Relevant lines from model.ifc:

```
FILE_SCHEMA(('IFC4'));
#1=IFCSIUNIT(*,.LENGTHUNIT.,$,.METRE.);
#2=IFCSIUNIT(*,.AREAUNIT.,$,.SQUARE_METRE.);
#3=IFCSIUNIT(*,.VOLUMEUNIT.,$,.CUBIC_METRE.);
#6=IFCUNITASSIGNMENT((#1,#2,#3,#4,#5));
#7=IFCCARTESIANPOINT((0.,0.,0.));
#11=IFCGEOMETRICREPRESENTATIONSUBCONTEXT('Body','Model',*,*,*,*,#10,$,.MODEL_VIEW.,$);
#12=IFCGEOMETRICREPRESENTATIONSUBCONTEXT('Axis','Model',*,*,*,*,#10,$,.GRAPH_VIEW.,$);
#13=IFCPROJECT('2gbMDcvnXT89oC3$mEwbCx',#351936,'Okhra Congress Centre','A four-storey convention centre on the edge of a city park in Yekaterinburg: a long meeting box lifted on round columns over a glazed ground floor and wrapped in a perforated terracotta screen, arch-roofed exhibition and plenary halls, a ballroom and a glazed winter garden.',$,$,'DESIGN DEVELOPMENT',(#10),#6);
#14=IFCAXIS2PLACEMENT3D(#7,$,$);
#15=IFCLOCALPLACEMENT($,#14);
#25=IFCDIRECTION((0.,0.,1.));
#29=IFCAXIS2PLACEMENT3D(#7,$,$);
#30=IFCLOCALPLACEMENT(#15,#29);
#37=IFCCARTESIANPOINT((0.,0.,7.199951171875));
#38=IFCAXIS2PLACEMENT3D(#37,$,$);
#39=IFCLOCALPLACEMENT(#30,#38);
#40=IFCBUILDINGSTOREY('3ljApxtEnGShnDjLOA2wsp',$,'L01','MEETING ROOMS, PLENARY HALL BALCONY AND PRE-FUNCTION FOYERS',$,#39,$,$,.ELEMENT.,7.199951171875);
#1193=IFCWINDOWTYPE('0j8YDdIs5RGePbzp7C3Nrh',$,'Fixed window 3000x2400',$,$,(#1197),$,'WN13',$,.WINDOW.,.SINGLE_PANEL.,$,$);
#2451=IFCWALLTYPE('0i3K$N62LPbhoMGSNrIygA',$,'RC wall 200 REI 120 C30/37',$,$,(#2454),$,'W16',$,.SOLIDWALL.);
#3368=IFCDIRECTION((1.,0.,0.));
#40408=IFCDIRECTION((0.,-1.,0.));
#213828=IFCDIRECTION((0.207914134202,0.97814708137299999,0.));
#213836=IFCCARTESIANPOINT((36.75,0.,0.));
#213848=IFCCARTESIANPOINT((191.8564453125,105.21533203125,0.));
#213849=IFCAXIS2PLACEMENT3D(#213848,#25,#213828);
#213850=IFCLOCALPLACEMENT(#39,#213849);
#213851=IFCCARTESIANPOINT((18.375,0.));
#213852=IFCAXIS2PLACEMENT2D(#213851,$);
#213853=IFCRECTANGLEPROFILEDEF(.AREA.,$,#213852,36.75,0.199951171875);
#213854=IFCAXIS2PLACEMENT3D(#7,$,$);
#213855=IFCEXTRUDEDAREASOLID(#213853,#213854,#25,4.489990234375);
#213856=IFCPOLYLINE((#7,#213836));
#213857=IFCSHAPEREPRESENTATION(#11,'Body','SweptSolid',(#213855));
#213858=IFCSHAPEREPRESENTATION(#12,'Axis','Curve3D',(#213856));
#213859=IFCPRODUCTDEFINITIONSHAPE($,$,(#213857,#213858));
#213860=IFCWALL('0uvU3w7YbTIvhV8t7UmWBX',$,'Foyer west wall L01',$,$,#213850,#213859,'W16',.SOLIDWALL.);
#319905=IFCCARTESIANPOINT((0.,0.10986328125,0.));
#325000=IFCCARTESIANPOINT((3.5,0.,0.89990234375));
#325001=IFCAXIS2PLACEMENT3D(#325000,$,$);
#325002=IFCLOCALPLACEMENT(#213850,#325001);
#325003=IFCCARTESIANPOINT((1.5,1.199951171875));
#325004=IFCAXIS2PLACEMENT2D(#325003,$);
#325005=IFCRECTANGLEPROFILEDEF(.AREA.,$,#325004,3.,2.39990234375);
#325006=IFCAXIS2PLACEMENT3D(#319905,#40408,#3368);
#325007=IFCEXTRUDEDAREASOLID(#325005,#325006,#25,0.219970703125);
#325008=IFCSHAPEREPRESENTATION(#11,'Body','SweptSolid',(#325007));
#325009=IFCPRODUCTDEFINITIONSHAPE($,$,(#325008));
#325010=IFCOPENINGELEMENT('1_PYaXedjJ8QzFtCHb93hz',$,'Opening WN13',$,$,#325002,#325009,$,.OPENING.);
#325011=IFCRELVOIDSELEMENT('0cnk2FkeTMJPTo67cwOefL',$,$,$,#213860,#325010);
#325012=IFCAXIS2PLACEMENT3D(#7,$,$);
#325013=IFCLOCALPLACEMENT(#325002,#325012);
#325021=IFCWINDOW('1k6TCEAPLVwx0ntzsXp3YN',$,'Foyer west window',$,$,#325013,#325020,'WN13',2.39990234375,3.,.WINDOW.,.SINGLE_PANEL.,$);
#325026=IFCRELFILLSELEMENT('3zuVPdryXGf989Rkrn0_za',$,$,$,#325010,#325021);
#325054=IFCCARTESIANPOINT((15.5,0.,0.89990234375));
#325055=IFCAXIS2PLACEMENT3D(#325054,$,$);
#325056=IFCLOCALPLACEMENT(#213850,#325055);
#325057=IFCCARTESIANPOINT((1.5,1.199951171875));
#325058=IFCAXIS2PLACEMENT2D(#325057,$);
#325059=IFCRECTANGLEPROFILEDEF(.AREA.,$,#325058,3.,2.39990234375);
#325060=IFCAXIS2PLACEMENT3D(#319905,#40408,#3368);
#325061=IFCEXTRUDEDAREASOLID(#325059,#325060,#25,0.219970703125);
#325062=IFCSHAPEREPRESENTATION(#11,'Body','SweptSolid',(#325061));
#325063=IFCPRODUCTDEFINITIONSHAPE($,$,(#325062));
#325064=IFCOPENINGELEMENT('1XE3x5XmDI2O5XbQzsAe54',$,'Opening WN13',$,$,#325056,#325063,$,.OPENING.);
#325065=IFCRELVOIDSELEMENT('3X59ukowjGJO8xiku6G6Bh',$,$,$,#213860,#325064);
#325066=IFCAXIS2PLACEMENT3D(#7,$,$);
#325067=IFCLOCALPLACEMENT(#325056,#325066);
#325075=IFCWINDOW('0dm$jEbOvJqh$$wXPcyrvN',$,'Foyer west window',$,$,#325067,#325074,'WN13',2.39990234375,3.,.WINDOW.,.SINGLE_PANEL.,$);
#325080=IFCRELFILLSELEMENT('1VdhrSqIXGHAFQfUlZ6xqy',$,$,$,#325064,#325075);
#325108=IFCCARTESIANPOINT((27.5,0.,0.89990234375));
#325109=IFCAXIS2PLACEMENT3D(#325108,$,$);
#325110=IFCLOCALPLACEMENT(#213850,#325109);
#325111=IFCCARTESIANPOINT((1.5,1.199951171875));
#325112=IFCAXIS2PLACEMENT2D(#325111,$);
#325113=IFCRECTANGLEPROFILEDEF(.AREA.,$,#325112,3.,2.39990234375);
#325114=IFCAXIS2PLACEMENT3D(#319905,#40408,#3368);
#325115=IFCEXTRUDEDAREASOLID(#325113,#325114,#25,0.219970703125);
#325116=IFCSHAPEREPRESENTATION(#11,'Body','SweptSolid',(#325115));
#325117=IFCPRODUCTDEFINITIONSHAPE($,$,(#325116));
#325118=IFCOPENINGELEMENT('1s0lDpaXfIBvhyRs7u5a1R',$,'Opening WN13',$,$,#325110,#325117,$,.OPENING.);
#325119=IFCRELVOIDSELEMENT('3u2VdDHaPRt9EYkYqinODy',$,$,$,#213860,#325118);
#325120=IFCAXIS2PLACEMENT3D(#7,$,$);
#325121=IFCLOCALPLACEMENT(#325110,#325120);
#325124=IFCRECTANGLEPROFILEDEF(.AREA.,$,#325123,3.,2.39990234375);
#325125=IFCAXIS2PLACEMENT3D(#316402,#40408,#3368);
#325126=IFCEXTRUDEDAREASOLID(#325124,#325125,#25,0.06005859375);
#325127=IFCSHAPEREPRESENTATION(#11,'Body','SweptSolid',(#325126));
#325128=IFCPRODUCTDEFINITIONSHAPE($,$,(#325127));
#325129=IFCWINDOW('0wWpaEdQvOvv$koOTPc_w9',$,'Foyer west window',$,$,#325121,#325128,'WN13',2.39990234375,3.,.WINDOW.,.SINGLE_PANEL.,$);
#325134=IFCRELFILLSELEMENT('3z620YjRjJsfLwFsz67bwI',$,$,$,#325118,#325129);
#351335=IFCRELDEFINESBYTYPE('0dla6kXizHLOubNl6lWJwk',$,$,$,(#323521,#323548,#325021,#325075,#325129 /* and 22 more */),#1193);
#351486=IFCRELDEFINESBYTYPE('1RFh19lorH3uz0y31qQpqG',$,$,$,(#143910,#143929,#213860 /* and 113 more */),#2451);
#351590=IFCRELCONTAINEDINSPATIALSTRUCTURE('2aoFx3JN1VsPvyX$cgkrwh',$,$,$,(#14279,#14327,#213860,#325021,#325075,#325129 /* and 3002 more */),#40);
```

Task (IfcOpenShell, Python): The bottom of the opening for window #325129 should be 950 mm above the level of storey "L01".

```python
import numpy as np
import ifcopenshell
import ifcopenshell.api.geometry
import ifcopenshell.geom
import ifcopenshell.util.element
import ifcopenshell.util.placement
import ifcopenshell.util.shape
import ifcopenshell.util.unit

model = ifcopenshell.open("model.ifc")
unit_scale = ifcopenshell.util.unit.calculate_unit_scale(model)

window = model.by_guid("0wWpaEdQvOvv$koOTPc_w9")
opening = window.FillsVoids[0].RelatingOpeningElement
storey = ifcopenshell.util.element.get_container(window, ifc_class="IfcBuildingStorey")
level = ifcopenshell.util.placement.get_local_placement(storey.ObjectPlacement)[2, 3]

# The opening's origin need not be at the sill, so measure its lowest point.
shape = ifcopenshell.geom.create_shape(ifcopenshell.geom.settings(), opening)
bottom = ifcopenshell.util.shape.get_shape_bottom_elevation(shape, shape.geometry) / unit_scale
dz = level + 0.95 / unit_scale - bottom

shift = np.array([0.0, 0.0, dz])
# The window is placed relative to its opening, so it follows when the opening moves.
matrix = ifcopenshell.util.placement.get_local_placement(opening.ObjectPlacement)
matrix[:3, 3] += shift
ifcopenshell.api.geometry.edit_object_placement(
    model, product=opening, matrix=matrix, is_si=False, should_transform_children=True
)

print(f"moved by {dz * unit_scale:+.3f} m")

model.write("model_v2.ifc")
```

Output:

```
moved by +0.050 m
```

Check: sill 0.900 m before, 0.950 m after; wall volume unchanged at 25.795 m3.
